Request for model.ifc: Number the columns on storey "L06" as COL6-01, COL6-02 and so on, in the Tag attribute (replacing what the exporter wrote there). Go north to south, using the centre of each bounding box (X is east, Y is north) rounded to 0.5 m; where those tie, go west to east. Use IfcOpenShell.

First a look at what the model holds.

```python
import ifcopenshell
import ifcopenshell.util.element
import ifcopenshell.util.placement

model = ifcopenshell.open("model.ifc")
print(model.schema)
storey = next(s for s in model.by_type("IfcBuildingStorey") if s.Name == "L06")
columns = [e for e in ifcopenshell.util.element.get_decomposition(storey) if e.is_a("IfcColumn")]
for e in sorted(columns, key=lambda e: e.id()):
    origin = ifcopenshell.util.placement.get_local_placement(e.ObjectPlacement)[:3, 3]
    print(e.id(), e.Tag, e.Name, origin.round(2) + 0.0, sep=" | ")
```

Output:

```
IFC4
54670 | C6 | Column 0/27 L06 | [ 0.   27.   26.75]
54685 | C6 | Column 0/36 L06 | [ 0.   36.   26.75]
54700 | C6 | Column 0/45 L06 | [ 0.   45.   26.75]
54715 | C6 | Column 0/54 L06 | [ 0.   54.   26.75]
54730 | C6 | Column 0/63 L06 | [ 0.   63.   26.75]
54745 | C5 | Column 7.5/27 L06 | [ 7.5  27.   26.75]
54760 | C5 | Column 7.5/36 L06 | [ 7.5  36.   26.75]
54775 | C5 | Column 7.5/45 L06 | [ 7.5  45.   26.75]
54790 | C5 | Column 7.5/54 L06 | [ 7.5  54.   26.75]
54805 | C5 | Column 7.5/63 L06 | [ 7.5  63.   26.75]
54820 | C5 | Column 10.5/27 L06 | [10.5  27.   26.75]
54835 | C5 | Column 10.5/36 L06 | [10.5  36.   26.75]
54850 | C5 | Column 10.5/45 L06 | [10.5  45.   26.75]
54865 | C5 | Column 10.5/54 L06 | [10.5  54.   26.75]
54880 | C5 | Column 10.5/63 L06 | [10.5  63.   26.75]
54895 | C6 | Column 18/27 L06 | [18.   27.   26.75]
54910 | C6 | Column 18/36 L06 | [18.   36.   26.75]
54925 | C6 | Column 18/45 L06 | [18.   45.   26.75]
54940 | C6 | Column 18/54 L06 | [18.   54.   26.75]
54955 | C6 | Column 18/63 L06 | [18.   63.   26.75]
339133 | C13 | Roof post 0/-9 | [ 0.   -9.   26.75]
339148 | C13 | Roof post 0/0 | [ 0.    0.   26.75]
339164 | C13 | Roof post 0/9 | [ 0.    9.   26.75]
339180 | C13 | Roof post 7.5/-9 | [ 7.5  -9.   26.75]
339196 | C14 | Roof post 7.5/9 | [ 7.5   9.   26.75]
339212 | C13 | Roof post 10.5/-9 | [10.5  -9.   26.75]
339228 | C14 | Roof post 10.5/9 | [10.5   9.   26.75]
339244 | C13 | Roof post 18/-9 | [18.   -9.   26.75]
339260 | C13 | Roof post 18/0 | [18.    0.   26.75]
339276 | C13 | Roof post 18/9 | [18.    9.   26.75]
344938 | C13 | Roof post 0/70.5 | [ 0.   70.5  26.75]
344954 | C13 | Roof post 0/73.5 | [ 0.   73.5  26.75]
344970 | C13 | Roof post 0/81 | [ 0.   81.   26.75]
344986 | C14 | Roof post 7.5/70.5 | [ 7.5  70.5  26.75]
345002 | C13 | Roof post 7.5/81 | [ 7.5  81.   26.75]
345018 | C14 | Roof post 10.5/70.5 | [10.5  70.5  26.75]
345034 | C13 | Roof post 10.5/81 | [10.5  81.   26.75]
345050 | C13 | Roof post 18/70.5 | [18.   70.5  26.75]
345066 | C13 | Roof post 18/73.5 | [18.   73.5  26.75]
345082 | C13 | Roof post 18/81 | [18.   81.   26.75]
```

```python
import ifcopenshell
import ifcopenshell.geom
import ifcopenshell.util.element
import ifcopenshell.util.shape

model = ifcopenshell.open("model.ifc")
settings = ifcopenshell.geom.settings()
settings.set("use-world-coords", True)


def centre(element):
    shape = ifcopenshell.geom.create_shape(settings, element)
    return ifcopenshell.util.shape.get_bbox_centroid(shape.geometry)


storey = next(s for s in model.by_type("IfcBuildingStorey") if s.Name == "L06")
columns = [e for e in ifcopenshell.util.element.get_decomposition(storey) if e.is_a("IfcColumn")]

# Insertion points can sit at a corner or the storey origin, so sort by the geometry (in metres).
centres = {e: centre(e) for e in columns}
columns.sort(key=lambda e: (-round(centres[e][1] / 0.5), centres[e][0]))

for i, e in enumerate(columns, start=1):
    number = f"COL6-{i:02d}"
    e.Tag = number
    print(e.id(), number)

model.write("model_v2.ifc")
```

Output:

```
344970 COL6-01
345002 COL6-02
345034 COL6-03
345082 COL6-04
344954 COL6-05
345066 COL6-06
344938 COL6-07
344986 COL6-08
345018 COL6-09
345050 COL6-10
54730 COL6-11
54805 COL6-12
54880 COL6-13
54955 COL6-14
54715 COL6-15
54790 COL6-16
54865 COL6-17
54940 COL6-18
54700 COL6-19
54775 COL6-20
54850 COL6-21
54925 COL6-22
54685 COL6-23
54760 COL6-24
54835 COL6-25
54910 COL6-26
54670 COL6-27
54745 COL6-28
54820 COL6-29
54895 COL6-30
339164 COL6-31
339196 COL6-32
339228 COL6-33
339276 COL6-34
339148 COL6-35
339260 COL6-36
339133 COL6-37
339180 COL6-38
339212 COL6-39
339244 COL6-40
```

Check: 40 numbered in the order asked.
